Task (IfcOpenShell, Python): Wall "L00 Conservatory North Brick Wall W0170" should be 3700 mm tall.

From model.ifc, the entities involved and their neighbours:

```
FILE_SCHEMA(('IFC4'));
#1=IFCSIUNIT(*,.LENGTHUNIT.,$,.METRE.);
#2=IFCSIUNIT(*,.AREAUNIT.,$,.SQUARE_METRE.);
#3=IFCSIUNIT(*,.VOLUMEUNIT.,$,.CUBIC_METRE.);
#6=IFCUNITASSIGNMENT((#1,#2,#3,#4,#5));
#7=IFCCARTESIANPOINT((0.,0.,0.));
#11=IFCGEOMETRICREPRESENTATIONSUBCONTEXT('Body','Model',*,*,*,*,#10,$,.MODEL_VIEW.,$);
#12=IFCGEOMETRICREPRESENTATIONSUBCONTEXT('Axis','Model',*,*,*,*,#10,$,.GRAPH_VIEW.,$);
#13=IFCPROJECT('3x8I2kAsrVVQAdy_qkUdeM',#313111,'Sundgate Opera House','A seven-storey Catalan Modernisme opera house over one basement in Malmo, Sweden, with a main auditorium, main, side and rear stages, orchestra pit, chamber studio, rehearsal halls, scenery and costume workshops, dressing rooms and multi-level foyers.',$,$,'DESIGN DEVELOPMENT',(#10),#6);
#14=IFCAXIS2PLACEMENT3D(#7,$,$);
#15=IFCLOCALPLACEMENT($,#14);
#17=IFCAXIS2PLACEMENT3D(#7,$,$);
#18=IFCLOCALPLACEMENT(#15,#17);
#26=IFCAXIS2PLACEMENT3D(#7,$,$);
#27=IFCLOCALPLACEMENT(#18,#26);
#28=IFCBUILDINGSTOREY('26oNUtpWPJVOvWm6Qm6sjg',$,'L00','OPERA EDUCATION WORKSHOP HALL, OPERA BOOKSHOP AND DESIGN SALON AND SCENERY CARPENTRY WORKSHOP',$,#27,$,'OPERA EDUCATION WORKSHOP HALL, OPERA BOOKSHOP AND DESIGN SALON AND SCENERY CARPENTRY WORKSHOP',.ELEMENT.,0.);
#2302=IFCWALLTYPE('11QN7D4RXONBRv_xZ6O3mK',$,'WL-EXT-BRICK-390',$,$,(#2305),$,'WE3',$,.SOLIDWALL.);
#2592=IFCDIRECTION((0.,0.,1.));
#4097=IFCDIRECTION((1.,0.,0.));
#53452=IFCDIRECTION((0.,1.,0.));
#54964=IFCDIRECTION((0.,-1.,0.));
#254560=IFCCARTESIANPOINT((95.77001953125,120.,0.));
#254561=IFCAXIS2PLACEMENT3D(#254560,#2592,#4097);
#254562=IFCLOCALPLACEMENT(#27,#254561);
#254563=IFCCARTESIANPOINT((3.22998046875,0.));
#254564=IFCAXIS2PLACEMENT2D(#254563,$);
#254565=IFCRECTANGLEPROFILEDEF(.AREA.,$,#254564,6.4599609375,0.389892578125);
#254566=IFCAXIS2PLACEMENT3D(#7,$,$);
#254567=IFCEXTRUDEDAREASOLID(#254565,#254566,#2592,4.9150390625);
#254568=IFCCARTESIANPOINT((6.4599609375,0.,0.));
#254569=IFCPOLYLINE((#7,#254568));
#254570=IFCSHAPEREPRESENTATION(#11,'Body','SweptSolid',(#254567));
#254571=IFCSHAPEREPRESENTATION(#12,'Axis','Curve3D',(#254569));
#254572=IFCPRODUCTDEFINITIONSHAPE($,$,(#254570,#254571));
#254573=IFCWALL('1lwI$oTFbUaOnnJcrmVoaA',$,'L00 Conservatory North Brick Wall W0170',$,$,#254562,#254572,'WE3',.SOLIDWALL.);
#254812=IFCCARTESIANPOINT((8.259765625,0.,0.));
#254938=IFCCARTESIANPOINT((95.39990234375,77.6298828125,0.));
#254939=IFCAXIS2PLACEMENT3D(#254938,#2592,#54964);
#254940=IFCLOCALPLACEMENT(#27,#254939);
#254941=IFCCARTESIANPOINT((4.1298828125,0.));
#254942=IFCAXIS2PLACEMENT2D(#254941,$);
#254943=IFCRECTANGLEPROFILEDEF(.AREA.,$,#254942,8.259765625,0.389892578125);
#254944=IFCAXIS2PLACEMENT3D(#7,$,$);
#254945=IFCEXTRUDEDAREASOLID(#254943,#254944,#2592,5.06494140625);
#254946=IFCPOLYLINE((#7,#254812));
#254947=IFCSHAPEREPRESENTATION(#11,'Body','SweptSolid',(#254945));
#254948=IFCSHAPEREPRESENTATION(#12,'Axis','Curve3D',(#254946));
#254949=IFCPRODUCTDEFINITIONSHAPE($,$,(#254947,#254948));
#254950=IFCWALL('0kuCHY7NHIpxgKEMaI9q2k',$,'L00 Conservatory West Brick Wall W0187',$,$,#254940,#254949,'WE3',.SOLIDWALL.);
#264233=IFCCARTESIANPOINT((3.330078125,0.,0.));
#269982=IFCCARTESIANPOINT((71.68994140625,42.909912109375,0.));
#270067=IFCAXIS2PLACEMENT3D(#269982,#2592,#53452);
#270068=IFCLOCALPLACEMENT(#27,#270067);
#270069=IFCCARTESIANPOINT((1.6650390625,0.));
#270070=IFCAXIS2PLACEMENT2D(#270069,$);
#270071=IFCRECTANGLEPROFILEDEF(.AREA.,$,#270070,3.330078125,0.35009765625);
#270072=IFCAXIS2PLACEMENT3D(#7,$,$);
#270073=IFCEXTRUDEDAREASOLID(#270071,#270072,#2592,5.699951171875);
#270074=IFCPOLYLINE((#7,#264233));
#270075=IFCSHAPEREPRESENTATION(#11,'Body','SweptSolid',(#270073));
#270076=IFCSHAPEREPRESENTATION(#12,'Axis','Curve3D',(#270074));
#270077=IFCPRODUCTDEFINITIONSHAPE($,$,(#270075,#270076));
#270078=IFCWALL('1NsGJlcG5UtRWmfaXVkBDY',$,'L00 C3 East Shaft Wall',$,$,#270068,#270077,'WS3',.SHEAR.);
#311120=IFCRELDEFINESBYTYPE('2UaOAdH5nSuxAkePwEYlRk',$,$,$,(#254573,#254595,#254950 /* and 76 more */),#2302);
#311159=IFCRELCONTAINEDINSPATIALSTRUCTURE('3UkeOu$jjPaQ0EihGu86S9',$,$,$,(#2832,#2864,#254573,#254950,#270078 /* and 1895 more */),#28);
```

```python
import ifcopenshell
import ifcopenshell.geom
import ifcopenshell.util.representation
import ifcopenshell.util.shape
import ifcopenshell.util.unit

model = ifcopenshell.open("model.ifc")
unit_scale = ifcopenshell.util.unit.calculate_unit_scale(model)
settings = ifcopenshell.geom.settings()


def volume(element):
    """Net volume in cubic metres, openings subtracted."""
    shape = ifcopenshell.geom.create_shape(settings, element)
    return ifcopenshell.util.shape.get_volume(shape.geometry)


wall = model.by_guid("1lwI$oTFbUaOnnJcrmVoaA")
before = volume(wall)

body = ifcopenshell.util.representation.get_representation(wall, "Model", "Body")
solid = body.Items[0]
old_height = solid.Depth
solid.Depth = 3.7 / unit_scale
after = volume(wall)

print(f"height {old_height:g} -> {solid.Depth:g}, volume {before:.3f} -> {after:.3f} m3")

model.write("model_updated.ifc")
```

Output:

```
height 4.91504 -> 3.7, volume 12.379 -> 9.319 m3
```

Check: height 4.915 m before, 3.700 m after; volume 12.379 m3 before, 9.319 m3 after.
